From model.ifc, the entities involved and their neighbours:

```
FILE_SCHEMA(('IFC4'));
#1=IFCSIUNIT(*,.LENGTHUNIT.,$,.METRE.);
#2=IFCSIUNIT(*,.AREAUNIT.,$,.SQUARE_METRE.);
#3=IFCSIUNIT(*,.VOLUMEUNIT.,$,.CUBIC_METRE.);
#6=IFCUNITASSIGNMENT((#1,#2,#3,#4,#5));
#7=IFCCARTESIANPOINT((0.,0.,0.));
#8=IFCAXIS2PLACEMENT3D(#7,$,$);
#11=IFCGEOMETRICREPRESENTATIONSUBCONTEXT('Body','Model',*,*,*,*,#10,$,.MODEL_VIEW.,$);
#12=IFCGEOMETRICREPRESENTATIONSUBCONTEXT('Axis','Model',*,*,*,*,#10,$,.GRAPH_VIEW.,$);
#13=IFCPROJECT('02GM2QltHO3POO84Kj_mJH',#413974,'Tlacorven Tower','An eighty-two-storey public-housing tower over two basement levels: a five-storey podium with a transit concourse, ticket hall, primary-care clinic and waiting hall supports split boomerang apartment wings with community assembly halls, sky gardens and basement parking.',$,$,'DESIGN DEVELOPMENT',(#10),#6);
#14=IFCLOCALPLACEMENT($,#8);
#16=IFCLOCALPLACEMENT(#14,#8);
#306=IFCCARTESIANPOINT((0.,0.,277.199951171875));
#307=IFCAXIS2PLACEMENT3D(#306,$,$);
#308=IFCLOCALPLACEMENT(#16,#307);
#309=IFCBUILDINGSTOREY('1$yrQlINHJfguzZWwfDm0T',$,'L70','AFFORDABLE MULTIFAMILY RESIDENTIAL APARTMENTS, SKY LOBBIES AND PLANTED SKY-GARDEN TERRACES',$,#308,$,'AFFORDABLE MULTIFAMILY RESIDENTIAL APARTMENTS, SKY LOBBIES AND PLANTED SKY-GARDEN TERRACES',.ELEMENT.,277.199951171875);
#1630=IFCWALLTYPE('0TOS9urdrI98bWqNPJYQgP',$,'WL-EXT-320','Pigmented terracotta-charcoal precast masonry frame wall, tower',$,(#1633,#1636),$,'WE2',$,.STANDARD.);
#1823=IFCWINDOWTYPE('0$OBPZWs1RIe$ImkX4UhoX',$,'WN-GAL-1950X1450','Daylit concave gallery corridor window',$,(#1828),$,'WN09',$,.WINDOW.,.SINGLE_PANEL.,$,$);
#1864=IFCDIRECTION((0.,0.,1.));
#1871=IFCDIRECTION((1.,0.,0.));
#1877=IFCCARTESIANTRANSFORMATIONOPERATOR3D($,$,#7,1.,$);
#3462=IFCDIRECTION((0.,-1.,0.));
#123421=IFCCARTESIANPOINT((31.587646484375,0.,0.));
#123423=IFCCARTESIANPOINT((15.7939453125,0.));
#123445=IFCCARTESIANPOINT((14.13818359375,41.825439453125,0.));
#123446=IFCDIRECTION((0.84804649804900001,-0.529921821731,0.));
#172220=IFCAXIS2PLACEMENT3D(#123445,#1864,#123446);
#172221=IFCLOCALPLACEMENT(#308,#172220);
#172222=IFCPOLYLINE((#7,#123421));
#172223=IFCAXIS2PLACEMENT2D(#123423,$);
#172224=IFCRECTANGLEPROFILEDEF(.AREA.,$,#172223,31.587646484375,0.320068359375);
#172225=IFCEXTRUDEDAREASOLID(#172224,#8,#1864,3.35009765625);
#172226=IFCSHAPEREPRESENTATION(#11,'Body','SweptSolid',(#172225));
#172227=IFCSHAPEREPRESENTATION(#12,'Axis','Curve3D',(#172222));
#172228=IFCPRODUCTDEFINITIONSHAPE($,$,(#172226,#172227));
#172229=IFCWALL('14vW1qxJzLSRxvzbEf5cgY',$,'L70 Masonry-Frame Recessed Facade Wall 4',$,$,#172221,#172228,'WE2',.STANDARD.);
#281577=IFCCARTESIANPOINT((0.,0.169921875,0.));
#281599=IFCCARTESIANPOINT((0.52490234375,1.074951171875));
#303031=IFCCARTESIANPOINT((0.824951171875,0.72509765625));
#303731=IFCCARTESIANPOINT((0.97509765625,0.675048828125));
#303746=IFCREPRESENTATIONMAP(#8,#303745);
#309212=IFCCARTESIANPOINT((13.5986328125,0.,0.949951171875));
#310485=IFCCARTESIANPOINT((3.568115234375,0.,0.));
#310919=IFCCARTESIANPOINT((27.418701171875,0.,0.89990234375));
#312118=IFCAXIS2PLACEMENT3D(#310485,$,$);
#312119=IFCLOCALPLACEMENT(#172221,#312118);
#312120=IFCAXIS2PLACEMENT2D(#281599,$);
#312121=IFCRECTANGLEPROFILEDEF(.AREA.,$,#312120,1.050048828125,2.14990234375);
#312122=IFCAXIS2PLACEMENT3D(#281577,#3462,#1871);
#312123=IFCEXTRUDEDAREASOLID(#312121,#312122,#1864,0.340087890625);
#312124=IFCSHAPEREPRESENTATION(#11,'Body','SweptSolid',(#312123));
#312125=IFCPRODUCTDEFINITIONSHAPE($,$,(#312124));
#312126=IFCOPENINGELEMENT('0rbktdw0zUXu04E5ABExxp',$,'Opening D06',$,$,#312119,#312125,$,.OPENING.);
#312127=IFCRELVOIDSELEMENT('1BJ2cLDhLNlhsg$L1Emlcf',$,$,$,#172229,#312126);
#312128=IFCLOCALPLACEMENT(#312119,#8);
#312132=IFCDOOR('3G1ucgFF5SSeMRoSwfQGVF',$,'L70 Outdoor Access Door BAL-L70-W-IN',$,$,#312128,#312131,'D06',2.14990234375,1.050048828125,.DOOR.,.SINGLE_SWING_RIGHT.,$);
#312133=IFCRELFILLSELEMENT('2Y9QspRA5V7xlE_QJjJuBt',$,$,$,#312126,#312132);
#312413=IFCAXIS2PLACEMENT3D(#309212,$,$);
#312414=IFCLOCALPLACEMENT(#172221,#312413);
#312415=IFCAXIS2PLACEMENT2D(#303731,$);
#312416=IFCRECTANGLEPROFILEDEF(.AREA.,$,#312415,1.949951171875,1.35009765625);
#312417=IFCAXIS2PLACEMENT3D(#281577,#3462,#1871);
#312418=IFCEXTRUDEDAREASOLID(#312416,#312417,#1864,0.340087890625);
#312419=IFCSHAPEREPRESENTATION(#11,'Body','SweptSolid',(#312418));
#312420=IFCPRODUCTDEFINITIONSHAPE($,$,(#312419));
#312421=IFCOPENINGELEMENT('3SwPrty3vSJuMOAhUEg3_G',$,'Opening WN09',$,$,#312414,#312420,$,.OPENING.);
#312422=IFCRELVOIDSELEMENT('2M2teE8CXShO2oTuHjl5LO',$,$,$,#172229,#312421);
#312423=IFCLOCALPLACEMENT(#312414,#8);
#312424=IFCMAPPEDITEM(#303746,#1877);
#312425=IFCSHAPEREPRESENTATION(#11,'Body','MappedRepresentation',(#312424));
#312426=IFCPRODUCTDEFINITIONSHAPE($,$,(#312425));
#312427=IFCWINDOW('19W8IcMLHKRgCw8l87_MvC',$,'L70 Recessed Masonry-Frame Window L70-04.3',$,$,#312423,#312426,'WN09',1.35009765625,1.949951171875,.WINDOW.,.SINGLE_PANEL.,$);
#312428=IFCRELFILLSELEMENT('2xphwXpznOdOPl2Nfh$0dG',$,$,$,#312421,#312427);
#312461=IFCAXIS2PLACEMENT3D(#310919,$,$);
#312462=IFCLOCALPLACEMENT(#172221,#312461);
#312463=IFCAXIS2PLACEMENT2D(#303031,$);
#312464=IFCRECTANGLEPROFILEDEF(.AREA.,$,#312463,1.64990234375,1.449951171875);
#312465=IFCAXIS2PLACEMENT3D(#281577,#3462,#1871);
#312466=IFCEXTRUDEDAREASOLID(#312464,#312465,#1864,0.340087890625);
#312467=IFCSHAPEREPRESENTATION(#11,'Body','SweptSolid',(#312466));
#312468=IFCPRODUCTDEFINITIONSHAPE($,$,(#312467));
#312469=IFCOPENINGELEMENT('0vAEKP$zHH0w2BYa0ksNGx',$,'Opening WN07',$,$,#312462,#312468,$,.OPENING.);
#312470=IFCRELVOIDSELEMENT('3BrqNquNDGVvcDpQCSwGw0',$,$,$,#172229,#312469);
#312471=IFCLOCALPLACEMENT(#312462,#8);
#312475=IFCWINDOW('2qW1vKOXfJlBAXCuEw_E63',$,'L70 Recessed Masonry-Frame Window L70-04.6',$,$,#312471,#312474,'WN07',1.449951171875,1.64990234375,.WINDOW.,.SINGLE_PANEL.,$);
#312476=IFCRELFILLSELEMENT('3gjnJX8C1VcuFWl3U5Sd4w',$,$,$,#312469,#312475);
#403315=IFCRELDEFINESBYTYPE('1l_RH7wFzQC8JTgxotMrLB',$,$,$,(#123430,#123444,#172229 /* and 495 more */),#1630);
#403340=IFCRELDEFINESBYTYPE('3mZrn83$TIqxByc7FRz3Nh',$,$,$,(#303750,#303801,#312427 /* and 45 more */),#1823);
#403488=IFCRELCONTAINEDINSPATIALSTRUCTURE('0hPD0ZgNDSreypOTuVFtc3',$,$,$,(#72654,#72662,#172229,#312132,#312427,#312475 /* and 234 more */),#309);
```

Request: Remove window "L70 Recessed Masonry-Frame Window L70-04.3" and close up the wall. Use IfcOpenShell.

```python
import ifcopenshell
import ifcopenshell.api.feature
import ifcopenshell.api.root
import ifcopenshell.geom
import ifcopenshell.util.shape

model = ifcopenshell.open("model.ifc")
settings = ifcopenshell.geom.settings()


def volume(element):
    """Net volume in cubic metres, openings subtracted."""
    shape = ifcopenshell.geom.create_shape(settings, element)
    return ifcopenshell.util.shape.get_volume(shape.geometry)


window = model.by_id(312427)
opening = window.FillsVoids[0].RelatingOpeningElement
wall = opening.VoidsElements[0].RelatingBuildingElement
before = volume(wall)

ifcopenshell.api.root.remove_product(model, product=window)
ifcopenshell.api.feature.remove_feature(model, feature=opening)

after = volume(wall)

print(f"wall volume {before:.3f} -> {after:.3f} m3")

model.write("model_rev.ifc")
```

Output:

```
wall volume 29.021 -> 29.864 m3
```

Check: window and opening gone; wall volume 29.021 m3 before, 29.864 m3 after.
